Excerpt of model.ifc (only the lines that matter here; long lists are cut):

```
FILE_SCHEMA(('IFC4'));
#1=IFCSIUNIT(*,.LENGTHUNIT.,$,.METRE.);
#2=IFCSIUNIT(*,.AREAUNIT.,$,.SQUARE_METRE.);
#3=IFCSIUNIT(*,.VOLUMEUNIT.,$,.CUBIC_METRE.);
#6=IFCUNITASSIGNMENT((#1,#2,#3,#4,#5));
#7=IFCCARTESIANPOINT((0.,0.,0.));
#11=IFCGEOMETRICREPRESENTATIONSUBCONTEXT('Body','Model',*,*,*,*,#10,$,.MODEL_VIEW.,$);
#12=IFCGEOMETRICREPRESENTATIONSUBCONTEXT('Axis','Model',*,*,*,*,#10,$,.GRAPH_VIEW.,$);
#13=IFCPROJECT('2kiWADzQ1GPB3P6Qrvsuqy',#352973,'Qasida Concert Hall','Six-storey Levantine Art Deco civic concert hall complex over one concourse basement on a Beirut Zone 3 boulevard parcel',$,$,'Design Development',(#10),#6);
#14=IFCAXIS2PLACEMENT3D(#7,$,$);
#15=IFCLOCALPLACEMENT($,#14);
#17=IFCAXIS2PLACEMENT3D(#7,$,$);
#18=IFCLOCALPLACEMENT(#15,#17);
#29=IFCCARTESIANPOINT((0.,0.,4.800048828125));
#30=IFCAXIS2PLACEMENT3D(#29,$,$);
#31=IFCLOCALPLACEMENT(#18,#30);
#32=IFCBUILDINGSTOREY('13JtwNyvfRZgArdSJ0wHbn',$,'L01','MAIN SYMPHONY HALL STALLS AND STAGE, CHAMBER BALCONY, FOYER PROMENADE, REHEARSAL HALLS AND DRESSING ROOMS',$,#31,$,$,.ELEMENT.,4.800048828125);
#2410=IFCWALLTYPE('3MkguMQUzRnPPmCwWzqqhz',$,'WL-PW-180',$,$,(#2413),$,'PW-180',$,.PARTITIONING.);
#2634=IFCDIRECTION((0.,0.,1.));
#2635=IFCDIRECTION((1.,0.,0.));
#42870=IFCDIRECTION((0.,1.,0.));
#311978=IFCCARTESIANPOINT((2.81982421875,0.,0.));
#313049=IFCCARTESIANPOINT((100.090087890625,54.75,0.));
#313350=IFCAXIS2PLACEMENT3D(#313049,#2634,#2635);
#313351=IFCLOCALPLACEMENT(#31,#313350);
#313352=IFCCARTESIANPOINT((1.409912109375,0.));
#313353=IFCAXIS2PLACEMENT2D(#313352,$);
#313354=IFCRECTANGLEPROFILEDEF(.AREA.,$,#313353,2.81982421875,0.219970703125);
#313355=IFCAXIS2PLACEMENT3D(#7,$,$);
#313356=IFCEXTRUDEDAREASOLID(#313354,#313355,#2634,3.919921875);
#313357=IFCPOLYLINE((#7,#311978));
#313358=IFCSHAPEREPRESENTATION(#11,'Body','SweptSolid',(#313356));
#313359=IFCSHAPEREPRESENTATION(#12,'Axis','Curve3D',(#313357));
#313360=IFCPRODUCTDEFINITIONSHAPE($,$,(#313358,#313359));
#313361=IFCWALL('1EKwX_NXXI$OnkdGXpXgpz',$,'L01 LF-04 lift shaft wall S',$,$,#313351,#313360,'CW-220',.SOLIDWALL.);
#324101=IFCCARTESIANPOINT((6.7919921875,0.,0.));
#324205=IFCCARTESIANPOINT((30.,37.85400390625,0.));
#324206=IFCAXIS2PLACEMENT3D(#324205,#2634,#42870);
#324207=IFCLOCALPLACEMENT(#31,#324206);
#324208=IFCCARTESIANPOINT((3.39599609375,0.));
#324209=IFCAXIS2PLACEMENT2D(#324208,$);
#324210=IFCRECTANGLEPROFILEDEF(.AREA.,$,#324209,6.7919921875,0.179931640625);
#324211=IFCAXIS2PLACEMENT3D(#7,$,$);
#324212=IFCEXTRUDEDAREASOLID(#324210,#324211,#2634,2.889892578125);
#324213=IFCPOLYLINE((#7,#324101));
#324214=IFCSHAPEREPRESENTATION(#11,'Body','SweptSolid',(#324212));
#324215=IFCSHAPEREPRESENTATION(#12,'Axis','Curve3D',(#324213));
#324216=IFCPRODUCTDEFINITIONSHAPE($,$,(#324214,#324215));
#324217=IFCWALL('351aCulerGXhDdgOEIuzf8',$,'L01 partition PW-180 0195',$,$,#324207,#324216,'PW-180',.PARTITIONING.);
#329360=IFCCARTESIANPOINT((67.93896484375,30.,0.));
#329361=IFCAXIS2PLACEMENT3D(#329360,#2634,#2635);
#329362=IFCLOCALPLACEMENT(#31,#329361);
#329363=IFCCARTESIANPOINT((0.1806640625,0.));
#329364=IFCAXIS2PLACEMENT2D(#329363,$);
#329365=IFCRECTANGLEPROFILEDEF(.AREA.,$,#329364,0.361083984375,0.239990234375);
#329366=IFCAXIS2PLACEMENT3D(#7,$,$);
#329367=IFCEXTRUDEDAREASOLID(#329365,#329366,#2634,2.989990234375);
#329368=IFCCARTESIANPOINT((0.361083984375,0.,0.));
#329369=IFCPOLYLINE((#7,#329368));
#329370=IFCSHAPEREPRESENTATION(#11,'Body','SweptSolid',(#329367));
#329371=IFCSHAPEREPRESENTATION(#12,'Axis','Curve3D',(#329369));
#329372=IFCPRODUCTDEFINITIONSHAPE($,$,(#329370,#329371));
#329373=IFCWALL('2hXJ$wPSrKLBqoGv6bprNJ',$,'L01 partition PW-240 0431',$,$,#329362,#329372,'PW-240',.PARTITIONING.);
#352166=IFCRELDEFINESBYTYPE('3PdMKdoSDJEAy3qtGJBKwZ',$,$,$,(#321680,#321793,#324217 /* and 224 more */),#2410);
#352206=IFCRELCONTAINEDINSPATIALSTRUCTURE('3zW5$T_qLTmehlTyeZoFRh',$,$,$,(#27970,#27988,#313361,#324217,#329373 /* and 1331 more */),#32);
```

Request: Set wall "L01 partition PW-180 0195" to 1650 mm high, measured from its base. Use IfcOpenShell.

```python
import ifcopenshell
import ifcopenshell.geom
import ifcopenshell.util.representation
import ifcopenshell.util.shape
import ifcopenshell.util.unit

model = ifcopenshell.open("model.ifc")
unit_scale = ifcopenshell.util.unit.calculate_unit_scale(model)
settings = ifcopenshell.geom.settings()


def volume(element):
    """Net volume in cubic metres, openings subtracted."""
    shape = ifcopenshell.geom.create_shape(settings, element)
    return ifcopenshell.util.shape.get_volume(shape.geometry)


wall = model.by_id(324217)
before = volume(wall)

body = ifcopenshell.util.representation.get_representation(wall, "Model", "Body")
solid = body.Items[0]
old_height = solid.Depth
solid.Depth = 1.65 / unit_scale
after = volume(wall)

print(f"height {old_height:g} -> {solid.Depth:g}, volume {before:.3f} -> {after:.3f} m3")

model.write("model_v2.ifc")
```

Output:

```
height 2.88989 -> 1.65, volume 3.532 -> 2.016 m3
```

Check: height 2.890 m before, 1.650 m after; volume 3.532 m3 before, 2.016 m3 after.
